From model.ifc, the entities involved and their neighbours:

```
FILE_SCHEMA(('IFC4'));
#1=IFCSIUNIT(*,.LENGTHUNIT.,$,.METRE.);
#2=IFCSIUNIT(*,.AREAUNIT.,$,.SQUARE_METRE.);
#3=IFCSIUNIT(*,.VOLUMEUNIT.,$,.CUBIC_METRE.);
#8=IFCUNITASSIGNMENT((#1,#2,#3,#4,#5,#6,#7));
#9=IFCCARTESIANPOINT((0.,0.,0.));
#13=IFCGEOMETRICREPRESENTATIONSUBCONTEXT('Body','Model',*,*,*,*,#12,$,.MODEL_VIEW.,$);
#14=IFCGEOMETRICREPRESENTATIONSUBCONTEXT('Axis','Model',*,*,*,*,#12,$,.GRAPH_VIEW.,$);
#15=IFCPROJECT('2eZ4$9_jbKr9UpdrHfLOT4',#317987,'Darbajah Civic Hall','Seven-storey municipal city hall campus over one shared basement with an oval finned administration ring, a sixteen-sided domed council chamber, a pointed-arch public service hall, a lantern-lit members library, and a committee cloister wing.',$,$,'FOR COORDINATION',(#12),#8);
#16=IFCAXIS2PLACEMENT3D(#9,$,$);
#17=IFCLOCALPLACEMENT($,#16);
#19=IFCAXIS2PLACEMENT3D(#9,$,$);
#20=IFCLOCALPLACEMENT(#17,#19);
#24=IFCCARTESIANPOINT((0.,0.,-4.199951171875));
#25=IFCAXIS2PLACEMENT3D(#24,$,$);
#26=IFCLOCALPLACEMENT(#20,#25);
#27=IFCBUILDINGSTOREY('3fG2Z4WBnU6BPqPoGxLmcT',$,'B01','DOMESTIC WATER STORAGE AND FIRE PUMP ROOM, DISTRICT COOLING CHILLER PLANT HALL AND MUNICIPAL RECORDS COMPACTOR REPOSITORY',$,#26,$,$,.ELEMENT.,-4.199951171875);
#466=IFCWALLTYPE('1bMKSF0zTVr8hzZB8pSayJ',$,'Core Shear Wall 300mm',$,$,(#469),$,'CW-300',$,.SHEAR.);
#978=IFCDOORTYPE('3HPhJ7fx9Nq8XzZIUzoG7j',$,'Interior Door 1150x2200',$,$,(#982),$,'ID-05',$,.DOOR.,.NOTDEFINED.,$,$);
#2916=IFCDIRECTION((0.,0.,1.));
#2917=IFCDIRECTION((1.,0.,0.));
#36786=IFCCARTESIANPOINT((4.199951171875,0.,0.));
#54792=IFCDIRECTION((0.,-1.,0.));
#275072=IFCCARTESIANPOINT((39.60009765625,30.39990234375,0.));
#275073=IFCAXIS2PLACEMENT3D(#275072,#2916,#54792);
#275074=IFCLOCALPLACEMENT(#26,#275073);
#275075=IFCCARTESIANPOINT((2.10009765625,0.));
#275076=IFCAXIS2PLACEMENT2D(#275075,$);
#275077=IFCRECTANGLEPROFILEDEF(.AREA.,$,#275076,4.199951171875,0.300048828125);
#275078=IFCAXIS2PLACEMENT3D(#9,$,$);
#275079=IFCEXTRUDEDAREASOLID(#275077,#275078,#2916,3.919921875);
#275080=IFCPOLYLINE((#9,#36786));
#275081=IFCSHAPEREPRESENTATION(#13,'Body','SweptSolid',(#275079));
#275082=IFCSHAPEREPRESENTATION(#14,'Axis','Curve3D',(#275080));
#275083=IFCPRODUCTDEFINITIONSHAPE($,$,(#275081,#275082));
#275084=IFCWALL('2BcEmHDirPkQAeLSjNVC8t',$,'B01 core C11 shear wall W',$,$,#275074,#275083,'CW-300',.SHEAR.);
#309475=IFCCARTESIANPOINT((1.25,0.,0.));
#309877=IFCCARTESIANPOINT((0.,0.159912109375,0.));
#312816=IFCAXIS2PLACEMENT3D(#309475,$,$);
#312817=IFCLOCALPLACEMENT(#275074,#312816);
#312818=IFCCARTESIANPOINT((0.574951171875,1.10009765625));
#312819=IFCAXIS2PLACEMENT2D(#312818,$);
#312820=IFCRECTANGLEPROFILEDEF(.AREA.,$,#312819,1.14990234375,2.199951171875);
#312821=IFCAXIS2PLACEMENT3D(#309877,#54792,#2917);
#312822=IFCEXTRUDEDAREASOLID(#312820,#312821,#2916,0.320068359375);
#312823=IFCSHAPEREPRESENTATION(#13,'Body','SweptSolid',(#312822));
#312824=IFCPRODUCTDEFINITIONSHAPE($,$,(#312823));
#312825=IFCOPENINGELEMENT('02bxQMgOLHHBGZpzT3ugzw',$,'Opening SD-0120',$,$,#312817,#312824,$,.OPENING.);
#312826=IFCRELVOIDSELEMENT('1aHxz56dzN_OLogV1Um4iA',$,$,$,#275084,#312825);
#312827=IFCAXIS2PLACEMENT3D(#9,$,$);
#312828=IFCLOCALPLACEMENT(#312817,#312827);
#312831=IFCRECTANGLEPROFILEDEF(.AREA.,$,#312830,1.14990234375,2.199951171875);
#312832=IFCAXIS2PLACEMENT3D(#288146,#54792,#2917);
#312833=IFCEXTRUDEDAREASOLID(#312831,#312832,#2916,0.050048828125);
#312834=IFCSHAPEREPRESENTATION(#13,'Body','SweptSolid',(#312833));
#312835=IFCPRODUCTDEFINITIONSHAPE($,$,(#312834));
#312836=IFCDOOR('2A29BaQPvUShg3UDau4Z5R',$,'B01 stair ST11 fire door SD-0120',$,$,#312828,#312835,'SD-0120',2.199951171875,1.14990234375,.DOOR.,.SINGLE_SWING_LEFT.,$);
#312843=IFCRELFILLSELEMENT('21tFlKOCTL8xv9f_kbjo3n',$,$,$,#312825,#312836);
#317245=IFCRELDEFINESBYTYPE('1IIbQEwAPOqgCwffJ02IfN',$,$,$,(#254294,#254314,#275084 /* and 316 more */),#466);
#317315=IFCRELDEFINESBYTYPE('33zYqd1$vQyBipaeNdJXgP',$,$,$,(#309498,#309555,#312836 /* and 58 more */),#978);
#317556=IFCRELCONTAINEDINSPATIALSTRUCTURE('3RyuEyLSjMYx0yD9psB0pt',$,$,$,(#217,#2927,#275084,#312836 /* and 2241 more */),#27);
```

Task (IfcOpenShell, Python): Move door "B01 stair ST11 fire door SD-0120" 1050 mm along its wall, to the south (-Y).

```python
import ifcopenshell
import ifcopenshell.api.geometry
import ifcopenshell.util.placement

model = ifcopenshell.open("model.ifc")

door = model.by_guid("2A29BaQPvUShg3UDau4Z5R")
opening = door.FillsVoids[0].RelatingOpeningElement
wall = opening.VoidsElements[0].RelatingBuildingElement

wall_matrix = ifcopenshell.util.placement.get_local_placement(wall.ObjectPlacement)
shift = wall_matrix[:3, 0] * 1.05
before = ifcopenshell.util.placement.get_local_placement(door.ObjectPlacement)[:3, 3].copy()

# The door is placed relative to its opening, so it follows when the opening moves.
matrix = ifcopenshell.util.placement.get_local_placement(opening.ObjectPlacement)
matrix[:3, 3] += shift
ifcopenshell.api.geometry.edit_object_placement(
    model, product=opening, matrix=matrix, is_si=False, should_transform_children=True
)

after = ifcopenshell.util.placement.get_local_placement(door.ObjectPlacement)[:3, 3]
print("door moved by", (after - before).round(3) + 0.0)

model.write("model_updated.ifc")
```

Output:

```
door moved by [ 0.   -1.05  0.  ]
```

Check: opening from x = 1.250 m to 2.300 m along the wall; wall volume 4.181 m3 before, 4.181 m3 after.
